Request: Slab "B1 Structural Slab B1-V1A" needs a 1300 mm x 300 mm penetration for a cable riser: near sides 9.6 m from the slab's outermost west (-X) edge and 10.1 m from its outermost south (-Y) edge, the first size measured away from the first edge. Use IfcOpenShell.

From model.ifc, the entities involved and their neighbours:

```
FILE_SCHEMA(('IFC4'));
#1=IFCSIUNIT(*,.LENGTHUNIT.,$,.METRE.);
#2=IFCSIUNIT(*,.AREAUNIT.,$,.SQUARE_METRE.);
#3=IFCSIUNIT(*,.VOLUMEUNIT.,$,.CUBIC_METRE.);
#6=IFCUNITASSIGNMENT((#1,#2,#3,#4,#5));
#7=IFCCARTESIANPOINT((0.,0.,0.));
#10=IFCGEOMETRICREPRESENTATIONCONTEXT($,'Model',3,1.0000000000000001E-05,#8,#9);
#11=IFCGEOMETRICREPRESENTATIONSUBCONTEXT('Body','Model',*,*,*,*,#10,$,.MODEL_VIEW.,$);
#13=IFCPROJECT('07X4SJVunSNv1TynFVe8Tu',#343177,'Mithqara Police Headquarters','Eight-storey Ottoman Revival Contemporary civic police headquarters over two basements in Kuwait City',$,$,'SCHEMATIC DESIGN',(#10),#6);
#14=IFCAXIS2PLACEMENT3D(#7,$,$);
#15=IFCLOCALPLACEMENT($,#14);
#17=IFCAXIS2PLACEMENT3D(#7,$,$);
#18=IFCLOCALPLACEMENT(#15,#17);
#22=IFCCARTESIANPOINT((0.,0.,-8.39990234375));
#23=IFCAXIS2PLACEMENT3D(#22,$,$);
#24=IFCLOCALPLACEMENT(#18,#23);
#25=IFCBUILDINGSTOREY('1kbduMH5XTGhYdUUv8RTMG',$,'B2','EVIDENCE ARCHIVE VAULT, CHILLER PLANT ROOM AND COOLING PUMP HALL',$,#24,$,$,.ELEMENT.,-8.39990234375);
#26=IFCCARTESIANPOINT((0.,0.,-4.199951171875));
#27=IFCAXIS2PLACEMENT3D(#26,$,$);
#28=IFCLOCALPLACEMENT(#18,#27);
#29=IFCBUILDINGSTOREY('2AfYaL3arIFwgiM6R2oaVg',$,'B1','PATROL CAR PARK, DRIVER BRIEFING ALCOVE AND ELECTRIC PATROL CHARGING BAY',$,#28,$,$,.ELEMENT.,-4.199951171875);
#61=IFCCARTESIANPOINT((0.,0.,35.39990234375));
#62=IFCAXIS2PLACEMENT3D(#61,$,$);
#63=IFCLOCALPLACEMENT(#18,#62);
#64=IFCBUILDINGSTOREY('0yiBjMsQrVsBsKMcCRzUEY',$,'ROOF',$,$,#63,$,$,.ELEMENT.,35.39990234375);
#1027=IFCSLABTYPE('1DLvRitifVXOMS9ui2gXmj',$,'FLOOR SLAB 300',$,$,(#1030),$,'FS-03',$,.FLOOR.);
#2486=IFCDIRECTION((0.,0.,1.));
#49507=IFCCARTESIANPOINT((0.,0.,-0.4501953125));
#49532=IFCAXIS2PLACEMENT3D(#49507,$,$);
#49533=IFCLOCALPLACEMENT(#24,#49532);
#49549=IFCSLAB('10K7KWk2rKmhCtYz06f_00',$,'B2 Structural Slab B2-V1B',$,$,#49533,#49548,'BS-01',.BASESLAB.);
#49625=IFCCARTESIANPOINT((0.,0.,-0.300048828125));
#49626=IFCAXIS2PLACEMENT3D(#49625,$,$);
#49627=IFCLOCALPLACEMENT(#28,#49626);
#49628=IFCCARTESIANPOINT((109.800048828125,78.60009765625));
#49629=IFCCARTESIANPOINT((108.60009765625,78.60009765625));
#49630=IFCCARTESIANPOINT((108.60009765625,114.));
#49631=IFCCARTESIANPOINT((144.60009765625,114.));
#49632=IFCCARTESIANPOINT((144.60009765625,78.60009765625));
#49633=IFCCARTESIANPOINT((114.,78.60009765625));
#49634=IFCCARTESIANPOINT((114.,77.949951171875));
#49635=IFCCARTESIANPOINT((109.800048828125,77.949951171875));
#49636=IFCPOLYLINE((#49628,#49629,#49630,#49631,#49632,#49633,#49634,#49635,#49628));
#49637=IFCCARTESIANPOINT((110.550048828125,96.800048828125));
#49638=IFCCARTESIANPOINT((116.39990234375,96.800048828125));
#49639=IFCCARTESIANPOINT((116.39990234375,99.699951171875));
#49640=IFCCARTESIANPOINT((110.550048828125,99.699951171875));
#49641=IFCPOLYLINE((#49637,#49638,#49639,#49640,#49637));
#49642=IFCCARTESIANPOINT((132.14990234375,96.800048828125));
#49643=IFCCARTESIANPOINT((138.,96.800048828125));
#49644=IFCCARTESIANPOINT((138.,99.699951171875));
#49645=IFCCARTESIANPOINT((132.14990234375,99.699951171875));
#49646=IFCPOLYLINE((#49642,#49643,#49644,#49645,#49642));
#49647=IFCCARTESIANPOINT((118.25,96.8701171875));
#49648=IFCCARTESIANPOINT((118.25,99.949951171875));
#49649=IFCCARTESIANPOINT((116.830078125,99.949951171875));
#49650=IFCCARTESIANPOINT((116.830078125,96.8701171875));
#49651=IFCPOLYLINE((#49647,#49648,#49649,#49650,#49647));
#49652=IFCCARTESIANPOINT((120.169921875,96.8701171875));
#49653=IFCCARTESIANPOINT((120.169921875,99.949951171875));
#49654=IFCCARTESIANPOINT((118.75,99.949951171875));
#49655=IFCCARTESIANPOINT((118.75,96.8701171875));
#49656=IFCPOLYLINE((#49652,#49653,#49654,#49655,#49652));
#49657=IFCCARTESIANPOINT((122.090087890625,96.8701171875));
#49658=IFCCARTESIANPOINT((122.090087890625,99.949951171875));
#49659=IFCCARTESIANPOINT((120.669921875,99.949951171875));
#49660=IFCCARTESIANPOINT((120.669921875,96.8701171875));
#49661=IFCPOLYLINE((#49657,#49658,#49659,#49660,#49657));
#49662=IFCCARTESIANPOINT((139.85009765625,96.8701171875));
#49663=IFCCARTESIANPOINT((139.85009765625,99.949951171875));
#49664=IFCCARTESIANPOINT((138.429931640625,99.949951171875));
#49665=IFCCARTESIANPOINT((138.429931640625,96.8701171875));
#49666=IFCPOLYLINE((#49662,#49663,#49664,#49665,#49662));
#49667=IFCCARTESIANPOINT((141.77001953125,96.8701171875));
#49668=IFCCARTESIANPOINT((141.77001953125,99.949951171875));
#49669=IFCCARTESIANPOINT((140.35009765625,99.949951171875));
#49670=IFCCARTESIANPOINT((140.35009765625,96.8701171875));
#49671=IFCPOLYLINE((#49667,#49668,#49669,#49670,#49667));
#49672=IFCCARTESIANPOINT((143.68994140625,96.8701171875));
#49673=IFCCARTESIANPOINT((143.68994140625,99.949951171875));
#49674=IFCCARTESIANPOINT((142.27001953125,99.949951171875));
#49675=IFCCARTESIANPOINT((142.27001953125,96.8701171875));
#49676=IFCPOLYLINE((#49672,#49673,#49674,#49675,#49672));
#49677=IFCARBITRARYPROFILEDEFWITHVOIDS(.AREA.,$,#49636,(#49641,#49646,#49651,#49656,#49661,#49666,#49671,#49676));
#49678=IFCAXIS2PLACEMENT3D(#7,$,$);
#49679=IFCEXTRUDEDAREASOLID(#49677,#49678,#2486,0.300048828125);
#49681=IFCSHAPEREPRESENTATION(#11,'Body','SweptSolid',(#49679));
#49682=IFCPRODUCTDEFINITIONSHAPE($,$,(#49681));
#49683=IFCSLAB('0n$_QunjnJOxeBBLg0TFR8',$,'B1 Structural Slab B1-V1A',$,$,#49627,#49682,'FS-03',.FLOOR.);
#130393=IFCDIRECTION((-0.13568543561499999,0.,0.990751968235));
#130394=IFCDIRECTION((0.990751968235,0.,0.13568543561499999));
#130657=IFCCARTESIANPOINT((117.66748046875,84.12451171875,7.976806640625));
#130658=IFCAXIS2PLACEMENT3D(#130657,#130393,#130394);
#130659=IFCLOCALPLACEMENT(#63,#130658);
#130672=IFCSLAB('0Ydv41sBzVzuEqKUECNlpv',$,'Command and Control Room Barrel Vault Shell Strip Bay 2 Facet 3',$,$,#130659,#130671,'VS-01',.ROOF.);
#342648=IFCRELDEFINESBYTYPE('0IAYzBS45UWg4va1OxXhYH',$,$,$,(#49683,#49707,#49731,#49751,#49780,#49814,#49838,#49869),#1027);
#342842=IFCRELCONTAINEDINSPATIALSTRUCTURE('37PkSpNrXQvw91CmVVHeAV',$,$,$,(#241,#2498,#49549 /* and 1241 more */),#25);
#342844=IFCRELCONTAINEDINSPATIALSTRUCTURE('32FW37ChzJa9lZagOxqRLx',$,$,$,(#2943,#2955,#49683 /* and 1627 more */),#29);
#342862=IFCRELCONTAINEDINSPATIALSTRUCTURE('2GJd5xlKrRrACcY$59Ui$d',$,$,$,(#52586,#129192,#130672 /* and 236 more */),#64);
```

```python
import numpy as np
import ifcopenshell
import ifcopenshell.api.feature
import ifcopenshell.api.geometry
import ifcopenshell.api.root
import ifcopenshell.geom
import ifcopenshell.util.placement
import ifcopenshell.util.representation
import ifcopenshell.util.shape
import ifcopenshell.util.unit

model = ifcopenshell.open("model.ifc")
unit_scale = ifcopenshell.util.unit.calculate_unit_scale(model)
settings = ifcopenshell.geom.settings()


def volume(element):
    """Net volume in cubic metres, openings subtracted."""
    shape = ifcopenshell.geom.create_shape(settings, element)
    return ifcopenshell.util.shape.get_volume(shape.geometry)


slab = model.by_guid("0n$_QunjnJOxeBBLg0TFR8")
before = volume(slab)

# Extent in the slab's own axes, in metres. The edges named are its -X and -Y sides.
slab_shape = ifcopenshell.geom.create_shape(settings, slab)
vertices = ifcopenshell.util.shape.get_vertices(slab_shape.geometry)
x_min, y_min, bottom = vertices.min(axis=0)
top = vertices[:, 2].max()

opening = ifcopenshell.api.root.create_entity(model, ifc_class="IfcOpeningElement", name="Cable riser opening", predefined_type="OPENING")
context = ifcopenshell.util.representation.get_context(model, "Model", "Body", "MODEL_VIEW")
width, depth = 1.3, 0.3
outline = [(0.0, 0.0), (width, 0.0), (width, depth), (0.0, depth), (0.0, 0.0)]
# Overshoot both faces by 50 mm so the cut is clean.
shape = ifcopenshell.api.geometry.add_slab_representation(
    model, context=context, depth=top - bottom + 0.1, polyline=outline
)
ifcopenshell.api.geometry.assign_representation(model, product=opening, representation=shape)

matrix = ifcopenshell.util.placement.get_local_placement(slab.ObjectPlacement)
matrix[:, 3] = matrix @ np.append(np.array([x_min + 9.6, y_min + 10.1, bottom - 0.05]) / unit_scale, 1.0)
ifcopenshell.api.geometry.edit_object_placement(model, product=opening, matrix=matrix, is_si=False)
ifcopenshell.api.feature.add_feature(model, feature=opening, element=slab)

after = volume(slab)

print(f"slab volume {before:.3f} -> {after:.3f} m3")

model.write("model_v2.ifc")
```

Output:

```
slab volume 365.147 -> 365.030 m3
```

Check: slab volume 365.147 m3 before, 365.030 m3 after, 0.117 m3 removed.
